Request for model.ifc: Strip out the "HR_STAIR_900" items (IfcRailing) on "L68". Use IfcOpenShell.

First a look at what the model holds.

```python
import ifcopenshell
import ifcopenshell.util.element

model = ifcopenshell.open("model.ifc")
print(model.schema)
storey = next(s for s in model.by_type("IfcBuildingStorey") if s.Name == "L68")
railings = [e for e in ifcopenshell.util.element.get_decomposition(storey) if e.is_a("IfcRailing")]
seen = {}
for e in railings:
    element_type = ifcopenshell.util.element.get_type(e)
    name = element_type.Name if element_type not in (None, e) else None
    seen[name] = seen.get(name, 0) + 1
for name, count in sorted(seen.items(), key=str):
    print(count, "x", name)
```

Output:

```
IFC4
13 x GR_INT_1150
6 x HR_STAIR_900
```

```python
import ifcopenshell
import ifcopenshell.api.root
import ifcopenshell.util.element

model = ifcopenshell.open("model.ifc")

storey = next(s for s in model.by_type("IfcBuildingStorey") if s.Name == "L68")
railings = [e for e in ifcopenshell.util.element.get_decomposition(storey) if e.is_a("IfcRailing")]
targets = [e for e in railings if (t := ifcopenshell.util.element.get_type(e)) not in (None, e) and t.Name == "HR_STAIR_900"]

for e in targets:
    ifcopenshell.api.root.remove_product(model, product=e)
print(len(targets), "removed")

model.write("model_edited.ifc")
```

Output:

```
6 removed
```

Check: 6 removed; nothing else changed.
